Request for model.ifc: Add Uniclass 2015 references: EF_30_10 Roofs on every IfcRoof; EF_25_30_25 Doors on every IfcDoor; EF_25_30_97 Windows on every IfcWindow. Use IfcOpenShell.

First a look at what the model holds.

```python
import ifcopenshell

model = ifcopenshell.open("model.ifc")
print(model.schema)
print("classifications:", [c.Name for c in model.by_type("IfcClassification")])
for ifc_class in ("IfcDoor", "IfcRoof", "IfcStair", "IfcWall", "IfcWindow"):
    print(ifc_class, len(model.by_type(ifc_class)))
```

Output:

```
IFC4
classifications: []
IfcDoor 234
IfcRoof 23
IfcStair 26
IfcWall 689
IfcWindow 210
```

```python
import ifcopenshell
import ifcopenshell.api.classification

model = ifcopenshell.open("model.ifc")

system = ifcopenshell.api.classification.add_classification(model, classification="Uniclass 2015")

codes = {
    "IfcRoof": ("EF_30_10", "Roofs"),
    "IfcDoor": ("EF_25_30_25", "Doors"),
    "IfcWindow": ("EF_25_30_97", "Windows"),
}
for ifc_class, (code, name) in codes.items():
    products = model.by_type(ifc_class)
    ifcopenshell.api.classification.add_reference(
        model, products=products, classification=system, identification=code, name=name
    )
    print(code, len(products))

model.write("model_edited.ifc")
```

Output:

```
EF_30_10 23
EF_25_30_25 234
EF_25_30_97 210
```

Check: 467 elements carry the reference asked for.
